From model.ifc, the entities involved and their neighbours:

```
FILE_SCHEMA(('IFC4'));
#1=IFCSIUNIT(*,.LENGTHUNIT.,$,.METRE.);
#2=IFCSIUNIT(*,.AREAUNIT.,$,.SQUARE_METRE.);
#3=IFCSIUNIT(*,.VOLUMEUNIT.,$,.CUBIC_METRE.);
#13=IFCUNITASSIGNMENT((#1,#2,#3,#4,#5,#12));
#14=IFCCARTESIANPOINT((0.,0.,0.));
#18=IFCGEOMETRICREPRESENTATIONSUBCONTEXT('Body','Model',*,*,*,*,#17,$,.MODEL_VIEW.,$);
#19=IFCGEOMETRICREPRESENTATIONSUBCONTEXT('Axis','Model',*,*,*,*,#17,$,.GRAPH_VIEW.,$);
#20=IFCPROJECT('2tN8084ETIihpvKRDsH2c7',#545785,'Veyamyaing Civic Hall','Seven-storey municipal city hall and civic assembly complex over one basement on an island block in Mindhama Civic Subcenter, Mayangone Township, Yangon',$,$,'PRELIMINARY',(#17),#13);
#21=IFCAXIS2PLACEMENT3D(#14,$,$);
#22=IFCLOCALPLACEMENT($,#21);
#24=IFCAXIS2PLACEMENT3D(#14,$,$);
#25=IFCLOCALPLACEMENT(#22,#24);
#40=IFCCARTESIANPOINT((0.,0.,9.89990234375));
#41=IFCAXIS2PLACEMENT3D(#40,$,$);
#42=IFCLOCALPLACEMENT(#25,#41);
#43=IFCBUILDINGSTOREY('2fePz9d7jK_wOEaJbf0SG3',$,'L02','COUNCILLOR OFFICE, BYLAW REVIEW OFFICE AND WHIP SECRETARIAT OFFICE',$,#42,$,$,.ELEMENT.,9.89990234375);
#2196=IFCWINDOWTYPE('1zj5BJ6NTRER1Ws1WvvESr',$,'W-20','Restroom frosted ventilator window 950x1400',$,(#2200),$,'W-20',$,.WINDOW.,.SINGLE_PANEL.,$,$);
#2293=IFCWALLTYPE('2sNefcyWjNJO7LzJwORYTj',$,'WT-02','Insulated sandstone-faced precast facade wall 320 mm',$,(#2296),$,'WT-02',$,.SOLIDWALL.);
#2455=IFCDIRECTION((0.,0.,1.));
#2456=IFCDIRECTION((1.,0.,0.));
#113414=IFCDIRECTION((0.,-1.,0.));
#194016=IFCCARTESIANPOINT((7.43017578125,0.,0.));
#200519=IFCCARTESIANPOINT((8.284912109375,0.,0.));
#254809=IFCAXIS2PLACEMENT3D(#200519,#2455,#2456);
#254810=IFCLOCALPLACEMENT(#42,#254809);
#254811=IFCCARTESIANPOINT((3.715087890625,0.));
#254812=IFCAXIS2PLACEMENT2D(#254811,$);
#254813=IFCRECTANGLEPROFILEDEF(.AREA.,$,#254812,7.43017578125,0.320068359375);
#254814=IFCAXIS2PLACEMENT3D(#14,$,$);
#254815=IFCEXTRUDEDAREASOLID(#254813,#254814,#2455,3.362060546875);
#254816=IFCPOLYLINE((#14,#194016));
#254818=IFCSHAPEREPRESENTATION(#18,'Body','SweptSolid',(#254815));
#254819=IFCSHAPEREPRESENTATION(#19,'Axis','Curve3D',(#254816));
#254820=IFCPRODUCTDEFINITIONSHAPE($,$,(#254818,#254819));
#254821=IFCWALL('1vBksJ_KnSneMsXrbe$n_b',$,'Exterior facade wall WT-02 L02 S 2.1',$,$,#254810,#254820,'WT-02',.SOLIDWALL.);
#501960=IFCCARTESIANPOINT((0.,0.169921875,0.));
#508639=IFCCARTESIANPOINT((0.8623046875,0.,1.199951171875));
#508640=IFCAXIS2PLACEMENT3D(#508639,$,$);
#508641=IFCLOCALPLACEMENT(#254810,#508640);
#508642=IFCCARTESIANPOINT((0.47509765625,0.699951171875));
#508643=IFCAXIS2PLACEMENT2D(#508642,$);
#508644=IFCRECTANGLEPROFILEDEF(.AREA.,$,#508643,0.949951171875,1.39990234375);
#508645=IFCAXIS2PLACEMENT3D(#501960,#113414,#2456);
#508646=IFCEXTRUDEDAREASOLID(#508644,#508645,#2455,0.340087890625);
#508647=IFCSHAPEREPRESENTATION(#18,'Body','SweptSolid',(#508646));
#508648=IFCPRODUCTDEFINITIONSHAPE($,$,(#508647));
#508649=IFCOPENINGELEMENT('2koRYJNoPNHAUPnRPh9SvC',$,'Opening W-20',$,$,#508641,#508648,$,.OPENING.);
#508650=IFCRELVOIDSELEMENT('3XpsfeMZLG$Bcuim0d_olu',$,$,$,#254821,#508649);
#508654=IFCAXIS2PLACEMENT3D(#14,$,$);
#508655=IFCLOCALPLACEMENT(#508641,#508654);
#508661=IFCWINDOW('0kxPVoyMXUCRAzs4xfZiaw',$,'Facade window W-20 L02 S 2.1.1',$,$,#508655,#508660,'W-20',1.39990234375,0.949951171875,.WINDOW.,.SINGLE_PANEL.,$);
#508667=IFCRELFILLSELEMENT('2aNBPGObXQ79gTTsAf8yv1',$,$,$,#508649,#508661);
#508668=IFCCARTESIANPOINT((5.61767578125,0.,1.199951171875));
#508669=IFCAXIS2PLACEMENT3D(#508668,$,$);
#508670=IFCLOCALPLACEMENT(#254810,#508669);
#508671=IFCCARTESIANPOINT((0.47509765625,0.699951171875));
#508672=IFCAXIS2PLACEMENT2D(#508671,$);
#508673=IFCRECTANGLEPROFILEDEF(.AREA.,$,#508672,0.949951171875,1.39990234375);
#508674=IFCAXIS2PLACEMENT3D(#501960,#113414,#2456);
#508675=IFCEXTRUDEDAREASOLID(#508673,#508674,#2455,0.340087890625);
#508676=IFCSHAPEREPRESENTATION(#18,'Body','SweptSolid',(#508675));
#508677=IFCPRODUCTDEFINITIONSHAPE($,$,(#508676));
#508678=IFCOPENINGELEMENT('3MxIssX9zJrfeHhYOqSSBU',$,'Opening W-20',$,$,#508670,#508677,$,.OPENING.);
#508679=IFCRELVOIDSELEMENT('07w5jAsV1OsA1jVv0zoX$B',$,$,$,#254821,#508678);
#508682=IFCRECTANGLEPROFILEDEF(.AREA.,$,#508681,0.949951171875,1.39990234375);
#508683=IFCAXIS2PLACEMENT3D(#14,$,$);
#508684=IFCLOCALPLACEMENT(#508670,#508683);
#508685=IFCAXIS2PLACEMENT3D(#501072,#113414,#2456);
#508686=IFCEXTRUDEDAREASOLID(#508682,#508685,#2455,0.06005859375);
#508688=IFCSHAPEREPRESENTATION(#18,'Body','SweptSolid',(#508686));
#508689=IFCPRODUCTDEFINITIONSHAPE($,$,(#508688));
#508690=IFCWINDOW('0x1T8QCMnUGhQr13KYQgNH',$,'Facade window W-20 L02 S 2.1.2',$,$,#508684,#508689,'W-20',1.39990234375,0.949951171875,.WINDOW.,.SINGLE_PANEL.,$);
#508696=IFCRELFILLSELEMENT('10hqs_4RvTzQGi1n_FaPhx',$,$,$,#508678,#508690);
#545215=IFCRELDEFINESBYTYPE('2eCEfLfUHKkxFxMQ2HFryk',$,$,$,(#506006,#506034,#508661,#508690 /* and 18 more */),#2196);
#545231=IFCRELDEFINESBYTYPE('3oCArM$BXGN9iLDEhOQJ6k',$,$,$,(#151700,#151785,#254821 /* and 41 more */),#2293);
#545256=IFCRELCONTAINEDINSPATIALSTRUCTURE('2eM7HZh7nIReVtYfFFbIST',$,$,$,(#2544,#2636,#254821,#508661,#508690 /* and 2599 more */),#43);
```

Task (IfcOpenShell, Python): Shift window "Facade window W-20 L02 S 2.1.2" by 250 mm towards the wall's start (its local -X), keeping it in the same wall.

```python
import ifcopenshell
import ifcopenshell.api.geometry
import ifcopenshell.util.placement
import ifcopenshell.util.unit

model = ifcopenshell.open("model.ifc")
unit_scale = ifcopenshell.util.unit.calculate_unit_scale(model)

window = model.by_id(508690)
opening = window.FillsVoids[0].RelatingOpeningElement
wall = opening.VoidsElements[0].RelatingBuildingElement

wall_matrix = ifcopenshell.util.placement.get_local_placement(wall.ObjectPlacement)
shift = wall_matrix[:3, 0] * -0.25 / unit_scale
before = ifcopenshell.util.placement.get_local_placement(window.ObjectPlacement)[:3, 3].copy()

# The window is placed relative to its opening, so it follows when the opening moves.
matrix = ifcopenshell.util.placement.get_local_placement(opening.ObjectPlacement)
matrix[:3, 3] += shift
ifcopenshell.api.geometry.edit_object_placement(
    model, product=opening, matrix=matrix, is_si=False, should_transform_children=True
)

after = ifcopenshell.util.placement.get_local_placement(window.ObjectPlacement)[:3, 3]
print("window moved by", (after - before).round(3) + 0.0)

model.write("model_v2.ifc")
```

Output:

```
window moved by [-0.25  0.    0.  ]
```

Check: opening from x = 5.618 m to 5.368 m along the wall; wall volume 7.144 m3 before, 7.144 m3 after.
